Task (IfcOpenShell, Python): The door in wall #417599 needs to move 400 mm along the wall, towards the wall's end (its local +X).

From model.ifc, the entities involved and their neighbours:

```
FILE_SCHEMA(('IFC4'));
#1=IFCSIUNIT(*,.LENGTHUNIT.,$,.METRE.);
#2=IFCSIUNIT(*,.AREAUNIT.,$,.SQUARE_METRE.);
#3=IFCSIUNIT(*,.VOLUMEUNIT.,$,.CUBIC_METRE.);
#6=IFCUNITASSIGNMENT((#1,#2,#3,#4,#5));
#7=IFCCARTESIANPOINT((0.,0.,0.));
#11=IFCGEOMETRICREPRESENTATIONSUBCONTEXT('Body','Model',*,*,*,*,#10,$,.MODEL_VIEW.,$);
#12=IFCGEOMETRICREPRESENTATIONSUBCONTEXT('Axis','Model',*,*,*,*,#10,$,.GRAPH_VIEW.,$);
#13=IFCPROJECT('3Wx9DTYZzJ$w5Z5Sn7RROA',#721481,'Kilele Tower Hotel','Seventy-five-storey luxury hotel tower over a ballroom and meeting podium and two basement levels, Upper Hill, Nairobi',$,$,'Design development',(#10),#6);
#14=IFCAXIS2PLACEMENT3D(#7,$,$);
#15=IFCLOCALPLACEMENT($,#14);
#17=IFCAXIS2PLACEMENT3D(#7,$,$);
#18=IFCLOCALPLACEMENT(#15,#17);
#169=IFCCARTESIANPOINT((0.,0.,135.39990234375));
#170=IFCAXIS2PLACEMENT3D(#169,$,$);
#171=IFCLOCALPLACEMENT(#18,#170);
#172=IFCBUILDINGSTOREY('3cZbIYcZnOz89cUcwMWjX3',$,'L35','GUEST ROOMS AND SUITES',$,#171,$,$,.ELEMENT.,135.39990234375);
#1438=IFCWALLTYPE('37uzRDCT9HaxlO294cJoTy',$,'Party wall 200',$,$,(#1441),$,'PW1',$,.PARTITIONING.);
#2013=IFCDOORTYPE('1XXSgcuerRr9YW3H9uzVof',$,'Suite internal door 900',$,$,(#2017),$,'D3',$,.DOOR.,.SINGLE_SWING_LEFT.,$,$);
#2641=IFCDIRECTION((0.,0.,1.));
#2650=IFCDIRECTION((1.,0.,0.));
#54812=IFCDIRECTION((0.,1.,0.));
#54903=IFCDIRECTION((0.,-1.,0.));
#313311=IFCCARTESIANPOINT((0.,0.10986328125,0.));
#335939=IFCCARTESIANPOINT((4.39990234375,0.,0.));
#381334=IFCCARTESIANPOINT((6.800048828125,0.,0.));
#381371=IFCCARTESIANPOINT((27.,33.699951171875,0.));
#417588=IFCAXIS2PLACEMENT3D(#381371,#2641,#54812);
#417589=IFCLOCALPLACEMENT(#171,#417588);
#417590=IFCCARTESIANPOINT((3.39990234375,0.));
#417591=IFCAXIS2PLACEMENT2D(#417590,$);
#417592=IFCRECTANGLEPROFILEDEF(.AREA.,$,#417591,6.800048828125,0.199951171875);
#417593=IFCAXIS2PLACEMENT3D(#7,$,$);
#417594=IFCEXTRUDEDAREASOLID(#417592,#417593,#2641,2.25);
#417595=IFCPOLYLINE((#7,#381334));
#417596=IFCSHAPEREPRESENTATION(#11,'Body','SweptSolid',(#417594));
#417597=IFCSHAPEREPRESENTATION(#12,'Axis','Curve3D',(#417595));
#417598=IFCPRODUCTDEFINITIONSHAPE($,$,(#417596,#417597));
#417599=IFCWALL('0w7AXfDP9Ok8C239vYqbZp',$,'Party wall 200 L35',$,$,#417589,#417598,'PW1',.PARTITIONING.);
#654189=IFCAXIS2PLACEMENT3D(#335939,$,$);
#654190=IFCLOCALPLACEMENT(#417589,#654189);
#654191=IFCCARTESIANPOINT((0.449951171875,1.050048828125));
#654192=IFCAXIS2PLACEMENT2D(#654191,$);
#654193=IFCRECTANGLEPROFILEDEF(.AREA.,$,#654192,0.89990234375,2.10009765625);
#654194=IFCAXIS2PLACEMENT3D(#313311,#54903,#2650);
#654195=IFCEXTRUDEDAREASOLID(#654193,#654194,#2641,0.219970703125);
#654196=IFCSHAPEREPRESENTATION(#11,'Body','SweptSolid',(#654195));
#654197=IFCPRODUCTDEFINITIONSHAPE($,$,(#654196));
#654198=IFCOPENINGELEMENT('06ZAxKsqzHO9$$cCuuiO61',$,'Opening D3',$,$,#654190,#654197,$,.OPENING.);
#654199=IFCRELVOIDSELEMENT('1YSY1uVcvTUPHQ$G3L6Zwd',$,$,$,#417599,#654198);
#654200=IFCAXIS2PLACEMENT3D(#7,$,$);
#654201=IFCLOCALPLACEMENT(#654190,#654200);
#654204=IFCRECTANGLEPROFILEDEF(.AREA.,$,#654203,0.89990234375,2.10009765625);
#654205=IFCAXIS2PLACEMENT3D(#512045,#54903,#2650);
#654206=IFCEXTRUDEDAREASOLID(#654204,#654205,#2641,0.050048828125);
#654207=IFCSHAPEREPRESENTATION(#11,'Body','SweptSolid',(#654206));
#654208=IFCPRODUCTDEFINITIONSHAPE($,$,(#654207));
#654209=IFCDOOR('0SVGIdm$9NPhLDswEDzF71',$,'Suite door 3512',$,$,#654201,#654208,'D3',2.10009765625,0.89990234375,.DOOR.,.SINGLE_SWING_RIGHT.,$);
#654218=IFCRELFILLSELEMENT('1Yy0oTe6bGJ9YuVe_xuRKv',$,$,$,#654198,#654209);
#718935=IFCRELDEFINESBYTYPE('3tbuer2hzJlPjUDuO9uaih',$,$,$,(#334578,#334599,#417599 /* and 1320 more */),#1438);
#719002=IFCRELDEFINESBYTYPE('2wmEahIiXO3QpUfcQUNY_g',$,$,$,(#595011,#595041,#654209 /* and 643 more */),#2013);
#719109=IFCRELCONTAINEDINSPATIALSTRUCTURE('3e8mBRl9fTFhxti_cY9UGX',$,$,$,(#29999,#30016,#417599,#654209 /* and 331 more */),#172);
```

```python
import ifcopenshell
import ifcopenshell.api.geometry
import ifcopenshell.util.placement

model = ifcopenshell.open("model.ifc")

door = model.by_guid("0SVGIdm$9NPhLDswEDzF71")
opening = door.FillsVoids[0].RelatingOpeningElement
wall = opening.VoidsElements[0].RelatingBuildingElement

wall_matrix = ifcopenshell.util.placement.get_local_placement(wall.ObjectPlacement)
shift = wall_matrix[:3, 0] * 0.4
before = ifcopenshell.util.placement.get_local_placement(door.ObjectPlacement)[:3, 3].copy()

# The door is placed relative to its opening, so it follows when the opening moves.
matrix = ifcopenshell.util.placement.get_local_placement(opening.ObjectPlacement)
matrix[:3, 3] += shift
ifcopenshell.api.geometry.edit_object_placement(
    model, product=opening, matrix=matrix, is_si=False, should_transform_children=True
)

after = ifcopenshell.util.placement.get_local_placement(door.ObjectPlacement)[:3, 3]
print("door moved by", (after - before).round(3) + 0.0)

model.write("model_updated.ifc")
```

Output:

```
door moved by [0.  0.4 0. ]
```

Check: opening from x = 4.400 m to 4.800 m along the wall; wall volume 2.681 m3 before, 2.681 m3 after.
